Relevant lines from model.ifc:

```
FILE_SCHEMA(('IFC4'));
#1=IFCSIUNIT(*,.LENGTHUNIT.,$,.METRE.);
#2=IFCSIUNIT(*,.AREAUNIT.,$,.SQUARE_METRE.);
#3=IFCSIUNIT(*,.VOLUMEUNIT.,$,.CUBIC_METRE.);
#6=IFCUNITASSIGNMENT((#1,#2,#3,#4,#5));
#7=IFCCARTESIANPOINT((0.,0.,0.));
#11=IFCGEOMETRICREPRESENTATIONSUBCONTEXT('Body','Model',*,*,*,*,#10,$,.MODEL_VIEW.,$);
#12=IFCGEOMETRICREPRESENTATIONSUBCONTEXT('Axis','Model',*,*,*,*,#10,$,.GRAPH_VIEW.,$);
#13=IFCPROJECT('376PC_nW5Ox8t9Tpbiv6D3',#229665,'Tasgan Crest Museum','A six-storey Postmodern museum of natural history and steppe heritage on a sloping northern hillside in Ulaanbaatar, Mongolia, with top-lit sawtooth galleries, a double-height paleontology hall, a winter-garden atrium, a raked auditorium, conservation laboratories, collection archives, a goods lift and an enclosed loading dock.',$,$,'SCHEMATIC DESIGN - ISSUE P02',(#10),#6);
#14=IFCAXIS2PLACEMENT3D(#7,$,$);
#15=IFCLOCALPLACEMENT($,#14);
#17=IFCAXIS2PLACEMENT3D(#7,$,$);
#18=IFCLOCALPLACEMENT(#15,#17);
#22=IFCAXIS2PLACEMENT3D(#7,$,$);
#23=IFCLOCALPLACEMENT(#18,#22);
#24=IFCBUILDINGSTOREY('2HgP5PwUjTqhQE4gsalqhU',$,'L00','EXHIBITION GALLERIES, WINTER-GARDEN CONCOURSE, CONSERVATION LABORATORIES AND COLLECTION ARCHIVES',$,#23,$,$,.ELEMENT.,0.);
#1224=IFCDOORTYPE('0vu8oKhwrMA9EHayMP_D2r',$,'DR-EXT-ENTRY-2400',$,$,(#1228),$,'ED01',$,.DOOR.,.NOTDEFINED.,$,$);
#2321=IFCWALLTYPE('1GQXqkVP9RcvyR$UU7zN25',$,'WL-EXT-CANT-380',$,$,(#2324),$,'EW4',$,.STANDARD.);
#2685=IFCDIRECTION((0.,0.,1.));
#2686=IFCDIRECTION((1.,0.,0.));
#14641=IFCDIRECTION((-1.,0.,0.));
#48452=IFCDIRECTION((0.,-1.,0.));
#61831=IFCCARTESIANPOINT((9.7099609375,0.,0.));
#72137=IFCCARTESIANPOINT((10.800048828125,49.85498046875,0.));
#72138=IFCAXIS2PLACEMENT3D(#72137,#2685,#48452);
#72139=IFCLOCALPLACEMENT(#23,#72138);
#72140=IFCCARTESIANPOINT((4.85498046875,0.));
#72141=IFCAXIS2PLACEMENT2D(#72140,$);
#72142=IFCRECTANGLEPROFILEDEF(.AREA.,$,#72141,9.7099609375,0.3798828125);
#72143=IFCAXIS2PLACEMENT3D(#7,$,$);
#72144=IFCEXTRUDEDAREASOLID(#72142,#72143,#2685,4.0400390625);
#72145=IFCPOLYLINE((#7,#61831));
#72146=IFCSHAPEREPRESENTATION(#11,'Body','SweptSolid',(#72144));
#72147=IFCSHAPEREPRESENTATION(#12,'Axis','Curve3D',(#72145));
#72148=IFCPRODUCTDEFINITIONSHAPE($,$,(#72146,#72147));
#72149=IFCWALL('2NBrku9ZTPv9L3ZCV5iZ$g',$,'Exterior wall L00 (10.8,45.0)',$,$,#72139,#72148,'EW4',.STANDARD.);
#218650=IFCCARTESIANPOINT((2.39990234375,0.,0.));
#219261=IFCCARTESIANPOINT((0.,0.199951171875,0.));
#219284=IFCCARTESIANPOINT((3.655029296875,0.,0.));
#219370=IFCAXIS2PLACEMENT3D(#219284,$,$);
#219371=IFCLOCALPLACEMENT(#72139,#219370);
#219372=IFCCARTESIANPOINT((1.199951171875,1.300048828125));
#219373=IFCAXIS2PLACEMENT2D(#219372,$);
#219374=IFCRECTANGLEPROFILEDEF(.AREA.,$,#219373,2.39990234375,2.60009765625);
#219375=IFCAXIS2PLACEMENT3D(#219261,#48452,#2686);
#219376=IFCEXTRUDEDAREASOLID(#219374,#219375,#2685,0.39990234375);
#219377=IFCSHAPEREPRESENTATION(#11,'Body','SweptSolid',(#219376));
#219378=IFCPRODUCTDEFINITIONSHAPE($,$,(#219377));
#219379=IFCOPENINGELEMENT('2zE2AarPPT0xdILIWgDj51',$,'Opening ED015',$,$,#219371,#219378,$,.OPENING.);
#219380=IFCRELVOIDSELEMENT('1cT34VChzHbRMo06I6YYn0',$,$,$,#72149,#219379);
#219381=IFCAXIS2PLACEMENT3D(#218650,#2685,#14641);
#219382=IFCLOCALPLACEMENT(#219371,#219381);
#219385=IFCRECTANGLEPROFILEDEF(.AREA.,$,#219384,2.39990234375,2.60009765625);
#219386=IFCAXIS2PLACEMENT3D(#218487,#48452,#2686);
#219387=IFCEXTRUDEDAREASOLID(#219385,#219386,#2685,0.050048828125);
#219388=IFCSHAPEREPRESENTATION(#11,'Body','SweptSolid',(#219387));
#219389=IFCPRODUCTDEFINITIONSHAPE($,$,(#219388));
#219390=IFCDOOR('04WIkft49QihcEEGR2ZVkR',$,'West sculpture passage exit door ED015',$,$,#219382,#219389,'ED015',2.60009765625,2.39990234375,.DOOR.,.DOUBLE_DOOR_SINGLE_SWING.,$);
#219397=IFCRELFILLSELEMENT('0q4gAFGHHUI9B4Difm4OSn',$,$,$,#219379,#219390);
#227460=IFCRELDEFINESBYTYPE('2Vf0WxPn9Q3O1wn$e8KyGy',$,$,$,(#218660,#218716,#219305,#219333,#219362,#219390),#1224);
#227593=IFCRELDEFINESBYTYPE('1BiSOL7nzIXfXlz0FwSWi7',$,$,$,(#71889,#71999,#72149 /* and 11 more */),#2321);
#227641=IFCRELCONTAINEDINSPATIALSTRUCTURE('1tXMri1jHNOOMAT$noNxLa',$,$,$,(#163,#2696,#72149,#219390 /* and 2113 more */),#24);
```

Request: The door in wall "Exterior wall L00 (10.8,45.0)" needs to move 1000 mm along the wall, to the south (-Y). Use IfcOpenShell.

```python
import ifcopenshell
import ifcopenshell.api.geometry
import ifcopenshell.util.placement

model = ifcopenshell.open("model.ifc")

door = model.by_guid("04WIkft49QihcEEGR2ZVkR")
opening = door.FillsVoids[0].RelatingOpeningElement
wall = opening.VoidsElements[0].RelatingBuildingElement

wall_matrix = ifcopenshell.util.placement.get_local_placement(wall.ObjectPlacement)
shift = wall_matrix[:3, 0] * 1.0
before = ifcopenshell.util.placement.get_local_placement(door.ObjectPlacement)[:3, 3].copy()

# The door is placed relative to its opening, so it follows when the opening moves.
matrix = ifcopenshell.util.placement.get_local_placement(opening.ObjectPlacement)
matrix[:3, 3] += shift
ifcopenshell.api.geometry.edit_object_placement(
    model, product=opening, matrix=matrix, is_si=False, should_transform_children=True
)

after = ifcopenshell.util.placement.get_local_placement(door.ObjectPlacement)[:3, 3]
print("door moved by", (after - before).round(3) + 0.0)

model.write("model-out.ifc")
```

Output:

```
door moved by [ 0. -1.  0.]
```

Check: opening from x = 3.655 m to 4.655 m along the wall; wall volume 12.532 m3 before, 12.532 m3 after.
